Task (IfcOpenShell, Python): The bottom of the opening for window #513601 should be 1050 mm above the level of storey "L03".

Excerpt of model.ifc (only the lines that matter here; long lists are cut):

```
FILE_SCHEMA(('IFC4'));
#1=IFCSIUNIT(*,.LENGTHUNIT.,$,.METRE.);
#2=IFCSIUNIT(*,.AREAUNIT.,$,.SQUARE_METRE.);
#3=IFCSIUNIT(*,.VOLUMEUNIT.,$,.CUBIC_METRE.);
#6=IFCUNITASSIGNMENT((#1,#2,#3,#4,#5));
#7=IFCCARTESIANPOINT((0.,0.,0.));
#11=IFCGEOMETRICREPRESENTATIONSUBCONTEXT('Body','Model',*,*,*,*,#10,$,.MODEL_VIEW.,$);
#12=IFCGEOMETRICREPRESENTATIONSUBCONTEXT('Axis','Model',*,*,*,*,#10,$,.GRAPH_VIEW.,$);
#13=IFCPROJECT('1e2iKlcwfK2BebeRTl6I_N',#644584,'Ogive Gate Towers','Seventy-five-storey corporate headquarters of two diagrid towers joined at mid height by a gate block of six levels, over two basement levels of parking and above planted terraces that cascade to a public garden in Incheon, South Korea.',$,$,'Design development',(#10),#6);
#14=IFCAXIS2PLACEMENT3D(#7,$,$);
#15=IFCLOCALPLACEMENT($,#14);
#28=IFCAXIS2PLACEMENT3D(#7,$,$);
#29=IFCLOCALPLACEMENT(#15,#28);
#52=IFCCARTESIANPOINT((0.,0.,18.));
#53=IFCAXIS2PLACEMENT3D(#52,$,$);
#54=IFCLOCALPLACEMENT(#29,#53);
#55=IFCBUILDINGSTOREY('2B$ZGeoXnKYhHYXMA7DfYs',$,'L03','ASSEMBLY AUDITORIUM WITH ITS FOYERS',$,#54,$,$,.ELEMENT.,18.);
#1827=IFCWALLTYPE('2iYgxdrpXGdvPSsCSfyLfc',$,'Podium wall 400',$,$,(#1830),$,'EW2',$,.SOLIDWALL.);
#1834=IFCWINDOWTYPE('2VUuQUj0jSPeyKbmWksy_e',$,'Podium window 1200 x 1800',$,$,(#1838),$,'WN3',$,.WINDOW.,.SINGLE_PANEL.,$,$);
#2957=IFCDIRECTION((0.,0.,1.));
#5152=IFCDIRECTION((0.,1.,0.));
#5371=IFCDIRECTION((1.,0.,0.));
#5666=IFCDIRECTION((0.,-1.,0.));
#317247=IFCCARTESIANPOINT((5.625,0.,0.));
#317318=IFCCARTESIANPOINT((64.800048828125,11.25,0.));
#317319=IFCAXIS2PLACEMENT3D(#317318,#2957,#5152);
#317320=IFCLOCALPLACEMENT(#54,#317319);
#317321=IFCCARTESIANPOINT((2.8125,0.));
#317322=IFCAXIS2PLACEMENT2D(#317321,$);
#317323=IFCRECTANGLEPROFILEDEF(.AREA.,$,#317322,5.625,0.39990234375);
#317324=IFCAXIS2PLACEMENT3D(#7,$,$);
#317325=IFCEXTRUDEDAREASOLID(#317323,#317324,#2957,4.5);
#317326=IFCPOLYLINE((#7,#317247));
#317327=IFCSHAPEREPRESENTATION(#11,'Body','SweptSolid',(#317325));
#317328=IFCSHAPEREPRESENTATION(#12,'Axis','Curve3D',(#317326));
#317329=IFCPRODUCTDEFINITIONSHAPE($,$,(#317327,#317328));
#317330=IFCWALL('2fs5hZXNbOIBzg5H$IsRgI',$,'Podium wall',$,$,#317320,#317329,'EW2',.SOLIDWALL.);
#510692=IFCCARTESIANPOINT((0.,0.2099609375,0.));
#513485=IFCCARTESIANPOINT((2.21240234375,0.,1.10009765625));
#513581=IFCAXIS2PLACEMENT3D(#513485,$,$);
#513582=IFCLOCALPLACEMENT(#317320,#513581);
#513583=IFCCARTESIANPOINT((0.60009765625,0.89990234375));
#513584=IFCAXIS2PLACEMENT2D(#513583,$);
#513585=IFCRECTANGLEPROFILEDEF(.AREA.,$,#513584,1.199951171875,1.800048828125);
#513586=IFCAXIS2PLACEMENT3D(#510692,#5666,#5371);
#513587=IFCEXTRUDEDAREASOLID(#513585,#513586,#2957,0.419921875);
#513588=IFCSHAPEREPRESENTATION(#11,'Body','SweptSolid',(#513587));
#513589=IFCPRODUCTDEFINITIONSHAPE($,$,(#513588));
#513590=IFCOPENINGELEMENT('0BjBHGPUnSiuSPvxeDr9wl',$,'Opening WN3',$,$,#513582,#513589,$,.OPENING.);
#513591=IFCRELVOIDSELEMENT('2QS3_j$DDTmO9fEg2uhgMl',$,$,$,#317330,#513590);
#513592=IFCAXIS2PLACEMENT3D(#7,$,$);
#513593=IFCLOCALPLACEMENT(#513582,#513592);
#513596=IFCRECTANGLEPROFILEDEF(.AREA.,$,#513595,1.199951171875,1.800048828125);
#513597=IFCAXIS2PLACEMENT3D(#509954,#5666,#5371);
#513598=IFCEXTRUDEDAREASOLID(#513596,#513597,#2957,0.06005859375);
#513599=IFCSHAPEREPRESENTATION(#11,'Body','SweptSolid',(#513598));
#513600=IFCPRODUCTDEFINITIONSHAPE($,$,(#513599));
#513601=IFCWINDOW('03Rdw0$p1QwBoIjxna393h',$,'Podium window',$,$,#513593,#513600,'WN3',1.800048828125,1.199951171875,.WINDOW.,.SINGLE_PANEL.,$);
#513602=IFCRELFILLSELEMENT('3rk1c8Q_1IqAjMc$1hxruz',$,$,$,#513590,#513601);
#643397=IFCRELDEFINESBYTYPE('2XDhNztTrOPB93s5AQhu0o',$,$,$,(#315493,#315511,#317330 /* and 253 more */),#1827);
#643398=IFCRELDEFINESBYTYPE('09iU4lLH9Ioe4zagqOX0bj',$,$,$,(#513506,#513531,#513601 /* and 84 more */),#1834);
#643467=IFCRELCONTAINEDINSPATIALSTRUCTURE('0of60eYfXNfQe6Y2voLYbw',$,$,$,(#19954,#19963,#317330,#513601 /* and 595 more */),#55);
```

```python
import numpy as np
import ifcopenshell
import ifcopenshell.api.geometry
import ifcopenshell.geom
import ifcopenshell.util.element
import ifcopenshell.util.placement
import ifcopenshell.util.shape
import ifcopenshell.util.unit

model = ifcopenshell.open("model.ifc")
unit_scale = ifcopenshell.util.unit.calculate_unit_scale(model)

window = model.by_guid("03Rdw0$p1QwBoIjxna393h")
opening = window.FillsVoids[0].RelatingOpeningElement
storey = ifcopenshell.util.element.get_container(window, ifc_class="IfcBuildingStorey")
level = ifcopenshell.util.placement.get_local_placement(storey.ObjectPlacement)[2, 3]

# The opening's origin need not be at the sill, so measure its lowest point.
shape = ifcopenshell.geom.create_shape(ifcopenshell.geom.settings(), opening)
bottom = ifcopenshell.util.shape.get_shape_bottom_elevation(shape, shape.geometry) / unit_scale
dz = level + 1.05 - bottom

shift = np.array([0.0, 0.0, dz])
# The window is placed relative to its opening, so it follows when the opening moves.
matrix = ifcopenshell.util.placement.get_local_placement(opening.ObjectPlacement)
matrix[:3, 3] += shift
ifcopenshell.api.geometry.edit_object_placement(
    model, product=opening, matrix=matrix, is_si=False, should_transform_children=True
)

print(f"moved by {dz * unit_scale:+.3f} m")

model.write("model_updated.ifc")
```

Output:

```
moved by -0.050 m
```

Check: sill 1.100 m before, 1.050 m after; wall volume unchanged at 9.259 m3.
